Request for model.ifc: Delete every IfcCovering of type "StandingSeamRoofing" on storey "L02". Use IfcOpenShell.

First a look at what the model holds.

```python
import ifcopenshell
import ifcopenshell.util.element

model = ifcopenshell.open("model.ifc")
print(model.schema)
storey = next(s for s in model.by_type("IfcBuildingStorey") if s.Name == "L02")
coverings = [e for e in ifcopenshell.util.element.get_decomposition(storey) if e.is_a("IfcCovering")]
seen = {}
for e in coverings:
    element_type = ifcopenshell.util.element.get_type(e)
    name = element_type.Name if element_type not in (None, e) else None
    seen[name] = seen.get(name, 0) + 1
for name, count in sorted(seen.items(), key=str):
    print(count, "x", name)
```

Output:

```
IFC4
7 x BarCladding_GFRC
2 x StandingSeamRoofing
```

```python
import ifcopenshell
import ifcopenshell.api.root
import ifcopenshell.util.element

model = ifcopenshell.open("model.ifc")

storey = next(s for s in model.by_type("IfcBuildingStorey") if s.Name == "L02")
coverings = [e for e in ifcopenshell.util.element.get_decomposition(storey) if e.is_a("IfcCovering")]
targets = [e for e in coverings if (t := ifcopenshell.util.element.get_type(e)) not in (None, e) and t.Name == "StandingSeamRoofing"]

for e in targets:
    ifcopenshell.api.root.remove_product(model, product=e)
print(len(targets), "removed")

model.write("model_edited.ifc")
```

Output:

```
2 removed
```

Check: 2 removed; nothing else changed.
